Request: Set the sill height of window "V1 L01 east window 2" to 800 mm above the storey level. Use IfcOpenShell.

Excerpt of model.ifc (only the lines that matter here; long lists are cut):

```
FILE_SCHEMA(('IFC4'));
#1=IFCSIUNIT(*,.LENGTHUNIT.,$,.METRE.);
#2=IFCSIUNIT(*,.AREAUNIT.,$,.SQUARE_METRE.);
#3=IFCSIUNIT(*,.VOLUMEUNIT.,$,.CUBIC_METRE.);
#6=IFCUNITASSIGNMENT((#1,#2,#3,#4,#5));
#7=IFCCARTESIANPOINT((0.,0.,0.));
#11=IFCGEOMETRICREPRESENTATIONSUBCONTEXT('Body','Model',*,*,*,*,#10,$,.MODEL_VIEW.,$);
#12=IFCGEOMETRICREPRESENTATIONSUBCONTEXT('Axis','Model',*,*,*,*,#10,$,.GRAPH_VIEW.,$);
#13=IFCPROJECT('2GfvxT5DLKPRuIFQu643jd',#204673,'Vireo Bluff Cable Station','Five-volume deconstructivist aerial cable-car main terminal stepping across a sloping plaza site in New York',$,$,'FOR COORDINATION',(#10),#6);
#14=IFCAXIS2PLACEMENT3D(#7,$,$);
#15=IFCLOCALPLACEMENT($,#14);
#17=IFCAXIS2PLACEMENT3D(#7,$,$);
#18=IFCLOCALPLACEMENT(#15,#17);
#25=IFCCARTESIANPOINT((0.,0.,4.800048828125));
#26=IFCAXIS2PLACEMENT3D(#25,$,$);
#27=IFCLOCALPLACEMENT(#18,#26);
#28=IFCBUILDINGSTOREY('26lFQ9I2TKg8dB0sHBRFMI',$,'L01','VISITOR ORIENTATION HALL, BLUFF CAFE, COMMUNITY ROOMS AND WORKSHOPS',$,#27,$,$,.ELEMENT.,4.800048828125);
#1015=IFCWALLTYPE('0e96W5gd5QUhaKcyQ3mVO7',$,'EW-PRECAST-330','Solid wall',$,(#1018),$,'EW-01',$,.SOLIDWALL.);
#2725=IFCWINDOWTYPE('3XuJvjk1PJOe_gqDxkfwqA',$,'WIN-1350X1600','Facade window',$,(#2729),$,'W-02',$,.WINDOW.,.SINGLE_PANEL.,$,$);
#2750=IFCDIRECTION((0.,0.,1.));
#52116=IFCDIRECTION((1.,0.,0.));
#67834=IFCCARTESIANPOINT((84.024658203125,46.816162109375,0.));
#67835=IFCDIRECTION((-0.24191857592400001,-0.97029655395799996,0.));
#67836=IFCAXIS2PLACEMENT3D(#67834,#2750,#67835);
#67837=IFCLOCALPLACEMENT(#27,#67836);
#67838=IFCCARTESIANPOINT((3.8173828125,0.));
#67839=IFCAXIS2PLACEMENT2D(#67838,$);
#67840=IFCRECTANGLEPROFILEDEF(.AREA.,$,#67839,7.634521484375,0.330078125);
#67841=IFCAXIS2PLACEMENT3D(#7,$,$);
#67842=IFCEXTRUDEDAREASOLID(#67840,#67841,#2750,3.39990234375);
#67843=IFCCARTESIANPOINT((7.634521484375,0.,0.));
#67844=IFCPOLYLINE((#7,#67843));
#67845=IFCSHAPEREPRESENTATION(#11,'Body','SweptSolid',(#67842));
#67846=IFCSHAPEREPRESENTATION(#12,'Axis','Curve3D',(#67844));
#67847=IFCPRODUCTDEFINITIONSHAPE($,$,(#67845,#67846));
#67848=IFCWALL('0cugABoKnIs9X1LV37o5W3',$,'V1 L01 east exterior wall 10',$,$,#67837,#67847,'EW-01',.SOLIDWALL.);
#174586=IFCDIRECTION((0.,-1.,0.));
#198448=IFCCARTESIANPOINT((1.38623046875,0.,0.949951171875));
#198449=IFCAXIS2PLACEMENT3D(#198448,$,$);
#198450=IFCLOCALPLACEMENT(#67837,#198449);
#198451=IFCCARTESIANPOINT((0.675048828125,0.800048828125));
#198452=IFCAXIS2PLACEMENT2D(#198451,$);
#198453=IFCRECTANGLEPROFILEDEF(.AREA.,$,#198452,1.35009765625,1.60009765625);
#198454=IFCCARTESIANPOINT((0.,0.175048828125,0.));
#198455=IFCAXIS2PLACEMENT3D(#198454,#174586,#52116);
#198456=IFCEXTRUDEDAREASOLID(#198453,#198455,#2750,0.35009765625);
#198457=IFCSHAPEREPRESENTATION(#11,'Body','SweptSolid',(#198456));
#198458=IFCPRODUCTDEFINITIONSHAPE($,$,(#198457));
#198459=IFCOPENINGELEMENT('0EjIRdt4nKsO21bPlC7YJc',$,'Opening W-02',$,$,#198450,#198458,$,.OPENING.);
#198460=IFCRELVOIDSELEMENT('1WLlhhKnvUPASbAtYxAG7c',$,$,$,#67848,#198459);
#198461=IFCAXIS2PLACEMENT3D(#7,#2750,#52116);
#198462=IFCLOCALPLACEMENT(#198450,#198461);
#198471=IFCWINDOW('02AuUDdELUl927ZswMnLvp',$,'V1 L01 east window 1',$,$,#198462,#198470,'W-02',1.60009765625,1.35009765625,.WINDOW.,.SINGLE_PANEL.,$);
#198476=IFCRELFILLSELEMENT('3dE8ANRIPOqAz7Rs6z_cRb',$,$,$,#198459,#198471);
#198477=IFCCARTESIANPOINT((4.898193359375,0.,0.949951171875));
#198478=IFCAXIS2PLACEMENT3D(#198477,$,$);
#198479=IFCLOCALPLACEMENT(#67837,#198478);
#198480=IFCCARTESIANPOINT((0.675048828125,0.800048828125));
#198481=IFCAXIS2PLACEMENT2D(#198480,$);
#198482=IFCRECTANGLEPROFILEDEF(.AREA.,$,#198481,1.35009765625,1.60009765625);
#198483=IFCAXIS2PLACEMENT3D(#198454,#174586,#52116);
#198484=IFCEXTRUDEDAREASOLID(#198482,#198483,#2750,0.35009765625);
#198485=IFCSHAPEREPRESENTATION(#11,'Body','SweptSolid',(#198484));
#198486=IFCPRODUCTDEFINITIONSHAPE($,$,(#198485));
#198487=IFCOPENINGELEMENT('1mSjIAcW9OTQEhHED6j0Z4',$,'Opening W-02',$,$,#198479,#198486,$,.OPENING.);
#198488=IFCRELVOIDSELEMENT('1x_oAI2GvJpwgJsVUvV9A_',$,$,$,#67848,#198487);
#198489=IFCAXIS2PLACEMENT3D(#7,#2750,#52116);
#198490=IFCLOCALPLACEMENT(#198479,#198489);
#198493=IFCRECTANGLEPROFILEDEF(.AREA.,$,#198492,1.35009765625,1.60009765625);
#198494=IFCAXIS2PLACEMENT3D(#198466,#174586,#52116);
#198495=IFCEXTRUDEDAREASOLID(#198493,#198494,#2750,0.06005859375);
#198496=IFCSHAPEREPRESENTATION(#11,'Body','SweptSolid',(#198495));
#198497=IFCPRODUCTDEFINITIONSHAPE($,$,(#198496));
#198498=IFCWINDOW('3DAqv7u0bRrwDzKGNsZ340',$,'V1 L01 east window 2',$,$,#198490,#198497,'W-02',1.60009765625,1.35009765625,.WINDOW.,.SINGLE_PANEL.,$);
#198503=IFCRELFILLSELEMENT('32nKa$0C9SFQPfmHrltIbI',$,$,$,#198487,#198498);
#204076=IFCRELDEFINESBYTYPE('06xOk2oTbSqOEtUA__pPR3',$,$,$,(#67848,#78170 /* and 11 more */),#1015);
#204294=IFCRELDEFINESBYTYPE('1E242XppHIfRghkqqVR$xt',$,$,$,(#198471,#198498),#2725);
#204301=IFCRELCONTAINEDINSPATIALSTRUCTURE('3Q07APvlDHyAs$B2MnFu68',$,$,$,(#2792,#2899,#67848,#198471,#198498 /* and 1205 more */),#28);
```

```python
import numpy as np
import ifcopenshell
import ifcopenshell.api.geometry
import ifcopenshell.geom
import ifcopenshell.util.element
import ifcopenshell.util.placement
import ifcopenshell.util.shape
import ifcopenshell.util.unit

model = ifcopenshell.open("model.ifc")
unit_scale = ifcopenshell.util.unit.calculate_unit_scale(model)

window = model.by_id(198498)
opening = window.FillsVoids[0].RelatingOpeningElement
storey = ifcopenshell.util.element.get_container(window, ifc_class="IfcBuildingStorey")
level = ifcopenshell.util.placement.get_local_placement(storey.ObjectPlacement)[2, 3]

# The opening's origin need not be at the sill, so measure its lowest point.
shape = ifcopenshell.geom.create_shape(ifcopenshell.geom.settings(), opening)
bottom = ifcopenshell.util.shape.get_shape_bottom_elevation(shape, shape.geometry) / unit_scale
dz = level + 0.8 - bottom

shift = np.array([0.0, 0.0, dz])
# The window is placed relative to its opening, so it follows when the opening moves.
matrix = ifcopenshell.util.placement.get_local_placement(opening.ObjectPlacement)
matrix[:3, 3] += shift
ifcopenshell.api.geometry.edit_object_placement(
    model, product=opening, matrix=matrix, is_si=False, should_transform_children=True
)

print(f"moved by {dz * unit_scale:+.3f} m")

model.write("model-out.ifc")
```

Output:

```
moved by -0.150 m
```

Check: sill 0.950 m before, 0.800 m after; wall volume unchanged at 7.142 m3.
